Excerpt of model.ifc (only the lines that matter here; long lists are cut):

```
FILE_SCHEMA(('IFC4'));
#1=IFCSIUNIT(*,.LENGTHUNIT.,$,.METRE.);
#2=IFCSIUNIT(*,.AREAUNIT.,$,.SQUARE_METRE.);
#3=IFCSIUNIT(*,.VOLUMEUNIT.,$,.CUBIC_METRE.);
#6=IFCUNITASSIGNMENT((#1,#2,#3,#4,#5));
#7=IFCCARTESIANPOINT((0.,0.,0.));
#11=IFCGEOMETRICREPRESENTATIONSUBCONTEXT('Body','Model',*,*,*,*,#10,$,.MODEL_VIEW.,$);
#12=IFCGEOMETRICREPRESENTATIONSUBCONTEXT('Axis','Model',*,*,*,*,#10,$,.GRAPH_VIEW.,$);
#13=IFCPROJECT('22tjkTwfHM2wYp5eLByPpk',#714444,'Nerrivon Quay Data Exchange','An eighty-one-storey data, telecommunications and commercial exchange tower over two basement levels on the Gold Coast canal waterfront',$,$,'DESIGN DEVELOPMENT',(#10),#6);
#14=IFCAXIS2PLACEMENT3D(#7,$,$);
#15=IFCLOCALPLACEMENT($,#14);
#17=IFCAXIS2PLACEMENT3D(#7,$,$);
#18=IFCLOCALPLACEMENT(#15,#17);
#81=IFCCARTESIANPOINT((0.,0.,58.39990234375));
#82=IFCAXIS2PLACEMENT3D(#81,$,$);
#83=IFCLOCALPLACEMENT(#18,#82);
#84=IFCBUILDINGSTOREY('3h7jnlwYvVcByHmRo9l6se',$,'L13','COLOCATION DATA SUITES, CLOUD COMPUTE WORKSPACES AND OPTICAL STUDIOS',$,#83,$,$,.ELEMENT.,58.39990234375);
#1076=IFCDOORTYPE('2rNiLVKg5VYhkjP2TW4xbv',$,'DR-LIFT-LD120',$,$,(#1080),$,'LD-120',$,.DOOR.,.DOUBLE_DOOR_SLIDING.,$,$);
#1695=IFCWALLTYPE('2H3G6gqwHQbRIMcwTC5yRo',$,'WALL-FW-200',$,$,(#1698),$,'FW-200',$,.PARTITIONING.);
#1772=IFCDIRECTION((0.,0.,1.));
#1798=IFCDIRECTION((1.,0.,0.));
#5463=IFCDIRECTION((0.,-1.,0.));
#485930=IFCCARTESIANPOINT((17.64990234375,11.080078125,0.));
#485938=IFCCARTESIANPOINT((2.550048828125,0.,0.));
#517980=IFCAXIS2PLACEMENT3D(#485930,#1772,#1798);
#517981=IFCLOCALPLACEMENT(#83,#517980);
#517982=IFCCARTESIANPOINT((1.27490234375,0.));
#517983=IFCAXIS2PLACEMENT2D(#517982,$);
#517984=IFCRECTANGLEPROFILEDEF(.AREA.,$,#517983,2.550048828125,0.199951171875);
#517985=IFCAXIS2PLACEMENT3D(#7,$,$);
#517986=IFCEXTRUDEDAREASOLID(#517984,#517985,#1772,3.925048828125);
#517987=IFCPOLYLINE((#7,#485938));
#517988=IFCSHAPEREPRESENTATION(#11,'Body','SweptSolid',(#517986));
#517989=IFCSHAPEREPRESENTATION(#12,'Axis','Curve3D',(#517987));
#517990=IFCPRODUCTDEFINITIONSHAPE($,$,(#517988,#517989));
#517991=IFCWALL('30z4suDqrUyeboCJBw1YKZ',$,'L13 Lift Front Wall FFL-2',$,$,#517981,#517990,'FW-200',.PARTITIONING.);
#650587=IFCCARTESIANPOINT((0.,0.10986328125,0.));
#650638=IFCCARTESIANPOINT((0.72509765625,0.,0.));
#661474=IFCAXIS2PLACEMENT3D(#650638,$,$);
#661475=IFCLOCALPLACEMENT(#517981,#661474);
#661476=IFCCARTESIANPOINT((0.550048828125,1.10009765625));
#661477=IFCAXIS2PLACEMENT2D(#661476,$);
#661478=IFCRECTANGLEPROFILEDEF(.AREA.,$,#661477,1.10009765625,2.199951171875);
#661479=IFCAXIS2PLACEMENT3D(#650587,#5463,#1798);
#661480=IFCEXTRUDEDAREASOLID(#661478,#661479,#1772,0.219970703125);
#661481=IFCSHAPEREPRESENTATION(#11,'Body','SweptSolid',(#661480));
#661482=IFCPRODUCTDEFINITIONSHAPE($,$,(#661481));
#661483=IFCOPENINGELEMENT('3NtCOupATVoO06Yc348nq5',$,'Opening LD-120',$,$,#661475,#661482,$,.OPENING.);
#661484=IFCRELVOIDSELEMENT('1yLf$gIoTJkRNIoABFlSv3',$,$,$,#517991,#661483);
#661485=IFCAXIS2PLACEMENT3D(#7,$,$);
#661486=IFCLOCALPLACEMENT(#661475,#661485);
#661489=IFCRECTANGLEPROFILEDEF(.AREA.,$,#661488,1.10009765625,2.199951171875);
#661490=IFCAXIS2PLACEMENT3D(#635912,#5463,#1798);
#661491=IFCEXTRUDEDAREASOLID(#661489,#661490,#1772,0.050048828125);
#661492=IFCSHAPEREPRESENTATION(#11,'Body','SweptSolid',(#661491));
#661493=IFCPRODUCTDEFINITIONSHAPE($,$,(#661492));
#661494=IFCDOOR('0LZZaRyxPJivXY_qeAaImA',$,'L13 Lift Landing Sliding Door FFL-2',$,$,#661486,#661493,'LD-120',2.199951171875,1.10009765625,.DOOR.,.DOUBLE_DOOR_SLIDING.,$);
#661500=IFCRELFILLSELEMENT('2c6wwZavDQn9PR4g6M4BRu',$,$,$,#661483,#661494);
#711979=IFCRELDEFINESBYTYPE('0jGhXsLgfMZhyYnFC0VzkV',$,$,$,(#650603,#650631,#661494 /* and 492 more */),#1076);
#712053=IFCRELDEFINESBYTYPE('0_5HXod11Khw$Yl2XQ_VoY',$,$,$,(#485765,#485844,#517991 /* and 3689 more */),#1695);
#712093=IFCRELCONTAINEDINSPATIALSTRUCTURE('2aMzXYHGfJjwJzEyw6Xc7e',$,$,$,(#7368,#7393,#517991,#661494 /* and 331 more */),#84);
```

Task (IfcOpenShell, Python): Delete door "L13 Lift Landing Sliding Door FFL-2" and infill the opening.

```python
import ifcopenshell
import ifcopenshell.api.feature
import ifcopenshell.api.root
import ifcopenshell.geom
import ifcopenshell.util.shape

model = ifcopenshell.open("model.ifc")
settings = ifcopenshell.geom.settings()


def volume(element):
    """Net volume in cubic metres, openings subtracted."""
    shape = ifcopenshell.geom.create_shape(settings, element)
    return ifcopenshell.util.shape.get_volume(shape.geometry)


door = model.by_id(661494)
opening = door.FillsVoids[0].RelatingOpeningElement
wall = opening.VoidsElements[0].RelatingBuildingElement
before = volume(wall)

ifcopenshell.api.root.remove_product(model, product=door)
ifcopenshell.api.feature.remove_feature(model, feature=opening)

after = volume(wall)

print(f"wall volume {before:.3f} -> {after:.3f} m3")

model.write("model_rev.ifc")
```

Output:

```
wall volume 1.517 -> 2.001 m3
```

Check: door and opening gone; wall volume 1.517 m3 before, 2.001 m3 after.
